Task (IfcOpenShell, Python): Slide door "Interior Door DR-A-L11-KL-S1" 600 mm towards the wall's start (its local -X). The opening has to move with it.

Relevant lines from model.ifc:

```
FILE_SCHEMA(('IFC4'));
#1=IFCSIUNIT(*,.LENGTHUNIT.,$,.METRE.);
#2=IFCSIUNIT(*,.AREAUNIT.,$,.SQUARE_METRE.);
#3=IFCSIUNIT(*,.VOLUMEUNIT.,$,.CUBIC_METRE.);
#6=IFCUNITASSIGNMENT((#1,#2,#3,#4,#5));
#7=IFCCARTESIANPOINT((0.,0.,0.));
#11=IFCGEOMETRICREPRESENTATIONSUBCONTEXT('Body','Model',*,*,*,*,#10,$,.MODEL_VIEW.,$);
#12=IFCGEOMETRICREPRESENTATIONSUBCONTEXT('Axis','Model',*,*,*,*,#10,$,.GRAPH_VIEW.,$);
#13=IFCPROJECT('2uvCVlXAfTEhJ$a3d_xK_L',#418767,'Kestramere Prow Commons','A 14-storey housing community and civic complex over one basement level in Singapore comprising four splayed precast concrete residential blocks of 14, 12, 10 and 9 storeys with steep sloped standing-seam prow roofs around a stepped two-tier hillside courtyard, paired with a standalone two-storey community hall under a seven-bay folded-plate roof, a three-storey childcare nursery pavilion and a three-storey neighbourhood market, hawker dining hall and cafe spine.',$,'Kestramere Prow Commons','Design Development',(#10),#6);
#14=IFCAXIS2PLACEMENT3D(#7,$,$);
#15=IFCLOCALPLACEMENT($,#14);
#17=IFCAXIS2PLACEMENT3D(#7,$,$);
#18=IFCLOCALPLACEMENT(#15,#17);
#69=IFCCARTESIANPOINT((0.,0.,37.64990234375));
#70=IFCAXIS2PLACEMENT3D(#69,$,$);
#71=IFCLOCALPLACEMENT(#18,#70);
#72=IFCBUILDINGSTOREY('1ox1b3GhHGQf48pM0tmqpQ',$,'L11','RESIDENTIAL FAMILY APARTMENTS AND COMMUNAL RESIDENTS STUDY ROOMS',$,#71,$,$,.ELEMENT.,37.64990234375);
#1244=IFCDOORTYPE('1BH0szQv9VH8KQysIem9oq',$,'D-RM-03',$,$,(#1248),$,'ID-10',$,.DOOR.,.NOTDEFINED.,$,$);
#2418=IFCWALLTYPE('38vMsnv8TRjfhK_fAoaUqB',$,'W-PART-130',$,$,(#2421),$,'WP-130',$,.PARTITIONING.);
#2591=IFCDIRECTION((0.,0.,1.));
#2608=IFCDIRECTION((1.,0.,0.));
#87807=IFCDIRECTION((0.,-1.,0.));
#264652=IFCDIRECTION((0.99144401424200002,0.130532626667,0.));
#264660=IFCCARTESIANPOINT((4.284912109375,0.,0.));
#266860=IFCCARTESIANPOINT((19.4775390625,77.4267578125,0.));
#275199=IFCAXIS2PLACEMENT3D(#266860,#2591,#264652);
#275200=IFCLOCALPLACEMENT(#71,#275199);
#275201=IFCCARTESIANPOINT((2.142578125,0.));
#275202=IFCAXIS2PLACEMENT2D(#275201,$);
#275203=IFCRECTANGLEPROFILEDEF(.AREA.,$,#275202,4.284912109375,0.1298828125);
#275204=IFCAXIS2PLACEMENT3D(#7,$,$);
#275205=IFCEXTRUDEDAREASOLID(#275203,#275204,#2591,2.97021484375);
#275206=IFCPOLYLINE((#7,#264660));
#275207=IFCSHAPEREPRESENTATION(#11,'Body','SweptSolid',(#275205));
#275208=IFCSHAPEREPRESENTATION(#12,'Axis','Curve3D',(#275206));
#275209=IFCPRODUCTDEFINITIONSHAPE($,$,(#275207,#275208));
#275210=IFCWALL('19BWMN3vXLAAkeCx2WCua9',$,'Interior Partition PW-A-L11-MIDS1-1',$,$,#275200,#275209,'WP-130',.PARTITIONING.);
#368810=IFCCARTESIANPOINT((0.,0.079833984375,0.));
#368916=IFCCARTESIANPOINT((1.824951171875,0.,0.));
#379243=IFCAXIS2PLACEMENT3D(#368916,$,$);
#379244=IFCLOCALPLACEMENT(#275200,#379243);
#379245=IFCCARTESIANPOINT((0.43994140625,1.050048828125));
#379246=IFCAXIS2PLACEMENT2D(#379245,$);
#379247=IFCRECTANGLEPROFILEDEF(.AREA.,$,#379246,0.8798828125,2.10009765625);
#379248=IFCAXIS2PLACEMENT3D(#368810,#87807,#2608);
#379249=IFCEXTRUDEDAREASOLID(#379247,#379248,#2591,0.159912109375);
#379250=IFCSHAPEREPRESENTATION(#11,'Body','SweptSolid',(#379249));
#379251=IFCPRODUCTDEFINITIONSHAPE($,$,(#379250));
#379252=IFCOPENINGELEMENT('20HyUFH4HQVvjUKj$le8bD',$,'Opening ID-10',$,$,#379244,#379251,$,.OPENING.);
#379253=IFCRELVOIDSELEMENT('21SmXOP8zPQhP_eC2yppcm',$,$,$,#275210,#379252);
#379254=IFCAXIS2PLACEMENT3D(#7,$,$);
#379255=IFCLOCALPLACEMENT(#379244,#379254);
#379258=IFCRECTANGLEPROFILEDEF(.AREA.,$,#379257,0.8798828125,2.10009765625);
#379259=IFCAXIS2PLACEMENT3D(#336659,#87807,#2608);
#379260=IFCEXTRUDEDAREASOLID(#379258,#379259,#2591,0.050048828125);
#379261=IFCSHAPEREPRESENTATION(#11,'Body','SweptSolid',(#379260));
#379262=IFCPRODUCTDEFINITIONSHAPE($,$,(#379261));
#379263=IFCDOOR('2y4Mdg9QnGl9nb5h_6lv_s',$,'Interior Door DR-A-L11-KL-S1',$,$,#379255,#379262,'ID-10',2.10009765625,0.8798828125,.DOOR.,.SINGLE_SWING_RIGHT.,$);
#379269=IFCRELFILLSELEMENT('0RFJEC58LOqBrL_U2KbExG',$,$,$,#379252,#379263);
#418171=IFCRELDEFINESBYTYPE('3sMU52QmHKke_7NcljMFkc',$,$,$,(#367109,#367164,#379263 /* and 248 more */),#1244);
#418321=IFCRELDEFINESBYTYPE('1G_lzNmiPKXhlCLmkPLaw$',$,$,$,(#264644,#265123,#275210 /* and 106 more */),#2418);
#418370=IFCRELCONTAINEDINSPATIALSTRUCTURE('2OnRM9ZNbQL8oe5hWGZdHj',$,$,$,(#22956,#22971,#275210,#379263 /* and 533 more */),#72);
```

```python
import ifcopenshell
import ifcopenshell.api.geometry
import ifcopenshell.util.placement
import ifcopenshell.util.unit

model = ifcopenshell.open("model.ifc")
unit_scale = ifcopenshell.util.unit.calculate_unit_scale(model)

door = model.by_id(379263)
opening = door.FillsVoids[0].RelatingOpeningElement
wall = opening.VoidsElements[0].RelatingBuildingElement

wall_matrix = ifcopenshell.util.placement.get_local_placement(wall.ObjectPlacement)
shift = wall_matrix[:3, 0] * -0.6 / unit_scale
before = ifcopenshell.util.placement.get_local_placement(door.ObjectPlacement)[:3, 3].copy()

# The door is placed relative to its opening, so it follows when the opening moves.
matrix = ifcopenshell.util.placement.get_local_placement(opening.ObjectPlacement)
matrix[:3, 3] += shift
ifcopenshell.api.geometry.edit_object_placement(
    model, product=opening, matrix=matrix, is_si=False, should_transform_children=True
)

after = ifcopenshell.util.placement.get_local_placement(door.ObjectPlacement)[:3, 3]
print("door moved by", (after - before).round(3) + 0.0)

model.write("model-out.ifc")
```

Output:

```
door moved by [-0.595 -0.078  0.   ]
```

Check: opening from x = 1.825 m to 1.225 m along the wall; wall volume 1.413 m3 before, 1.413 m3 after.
